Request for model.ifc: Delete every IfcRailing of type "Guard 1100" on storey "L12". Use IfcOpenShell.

First a look at what the model holds.

```python
import ifcopenshell
import ifcopenshell.util.element

model = ifcopenshell.open("model.ifc")
print(model.schema)
storey = next(s for s in model.by_type("IfcBuildingStorey") if s.Name == "L12")
railings = [e for e in ifcopenshell.util.element.get_decomposition(storey) if e.is_a("IfcRailing")]
seen = {}
for e in railings:
    element_type = ifcopenshell.util.element.get_type(e)
    name = element_type.Name if element_type not in (None, e) else None
    seen[name] = seen.get(name, 0) + 1
for name, count in sorted(seen.items(), key=str):
    print(count, "x", name)
```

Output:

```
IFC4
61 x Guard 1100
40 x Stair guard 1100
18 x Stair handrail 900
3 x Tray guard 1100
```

```python
import ifcopenshell
import ifcopenshell.api.root
import ifcopenshell.util.element

model = ifcopenshell.open("model.ifc")

storey = next(s for s in model.by_type("IfcBuildingStorey") if s.Name == "L12")
railings = [e for e in ifcopenshell.util.element.get_decomposition(storey) if e.is_a("IfcRailing")]
targets = [e for e in railings if (t := ifcopenshell.util.element.get_type(e)) not in (None, e) and t.Name == "Guard 1100"]

for e in targets:
    ifcopenshell.api.root.remove_product(model, product=e)
print(len(targets), "removed")

model.write("model_v2.ifc")
```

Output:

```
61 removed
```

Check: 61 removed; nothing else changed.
